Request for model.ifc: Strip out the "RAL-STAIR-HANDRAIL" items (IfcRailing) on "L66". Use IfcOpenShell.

First a look at what the model holds.

```python
import ifcopenshell
import ifcopenshell.util.element

model = ifcopenshell.open("model.ifc")
print(model.schema)
storey = next(s for s in model.by_type("IfcBuildingStorey") if s.Name == "L66")
railings = [e for e in ifcopenshell.util.element.get_decomposition(storey) if e.is_a("IfcRailing")]
seen = {}
for e in railings:
    element_type = ifcopenshell.util.element.get_type(e)
    name = element_type.Name if element_type not in (None, e) else None
    seen[name] = seen.get(name, 0) + 1
for name, count in sorted(seen.items(), key=str):
    print(count, "x", name)
```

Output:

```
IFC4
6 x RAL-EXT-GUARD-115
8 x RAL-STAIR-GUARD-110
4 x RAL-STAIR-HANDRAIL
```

```python
import ifcopenshell
import ifcopenshell.api.root
import ifcopenshell.util.element

model = ifcopenshell.open("model.ifc")

storey = next(s for s in model.by_type("IfcBuildingStorey") if s.Name == "L66")
railings = [e for e in ifcopenshell.util.element.get_decomposition(storey) if e.is_a("IfcRailing")]
targets = [e for e in railings if (t := ifcopenshell.util.element.get_type(e)) not in (None, e) and t.Name == "RAL-STAIR-HANDRAIL"]

for e in targets:
    ifcopenshell.api.root.remove_product(model, product=e)
print(len(targets), "removed")

model.write("model_v2.ifc")
```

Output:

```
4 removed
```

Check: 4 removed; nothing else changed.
